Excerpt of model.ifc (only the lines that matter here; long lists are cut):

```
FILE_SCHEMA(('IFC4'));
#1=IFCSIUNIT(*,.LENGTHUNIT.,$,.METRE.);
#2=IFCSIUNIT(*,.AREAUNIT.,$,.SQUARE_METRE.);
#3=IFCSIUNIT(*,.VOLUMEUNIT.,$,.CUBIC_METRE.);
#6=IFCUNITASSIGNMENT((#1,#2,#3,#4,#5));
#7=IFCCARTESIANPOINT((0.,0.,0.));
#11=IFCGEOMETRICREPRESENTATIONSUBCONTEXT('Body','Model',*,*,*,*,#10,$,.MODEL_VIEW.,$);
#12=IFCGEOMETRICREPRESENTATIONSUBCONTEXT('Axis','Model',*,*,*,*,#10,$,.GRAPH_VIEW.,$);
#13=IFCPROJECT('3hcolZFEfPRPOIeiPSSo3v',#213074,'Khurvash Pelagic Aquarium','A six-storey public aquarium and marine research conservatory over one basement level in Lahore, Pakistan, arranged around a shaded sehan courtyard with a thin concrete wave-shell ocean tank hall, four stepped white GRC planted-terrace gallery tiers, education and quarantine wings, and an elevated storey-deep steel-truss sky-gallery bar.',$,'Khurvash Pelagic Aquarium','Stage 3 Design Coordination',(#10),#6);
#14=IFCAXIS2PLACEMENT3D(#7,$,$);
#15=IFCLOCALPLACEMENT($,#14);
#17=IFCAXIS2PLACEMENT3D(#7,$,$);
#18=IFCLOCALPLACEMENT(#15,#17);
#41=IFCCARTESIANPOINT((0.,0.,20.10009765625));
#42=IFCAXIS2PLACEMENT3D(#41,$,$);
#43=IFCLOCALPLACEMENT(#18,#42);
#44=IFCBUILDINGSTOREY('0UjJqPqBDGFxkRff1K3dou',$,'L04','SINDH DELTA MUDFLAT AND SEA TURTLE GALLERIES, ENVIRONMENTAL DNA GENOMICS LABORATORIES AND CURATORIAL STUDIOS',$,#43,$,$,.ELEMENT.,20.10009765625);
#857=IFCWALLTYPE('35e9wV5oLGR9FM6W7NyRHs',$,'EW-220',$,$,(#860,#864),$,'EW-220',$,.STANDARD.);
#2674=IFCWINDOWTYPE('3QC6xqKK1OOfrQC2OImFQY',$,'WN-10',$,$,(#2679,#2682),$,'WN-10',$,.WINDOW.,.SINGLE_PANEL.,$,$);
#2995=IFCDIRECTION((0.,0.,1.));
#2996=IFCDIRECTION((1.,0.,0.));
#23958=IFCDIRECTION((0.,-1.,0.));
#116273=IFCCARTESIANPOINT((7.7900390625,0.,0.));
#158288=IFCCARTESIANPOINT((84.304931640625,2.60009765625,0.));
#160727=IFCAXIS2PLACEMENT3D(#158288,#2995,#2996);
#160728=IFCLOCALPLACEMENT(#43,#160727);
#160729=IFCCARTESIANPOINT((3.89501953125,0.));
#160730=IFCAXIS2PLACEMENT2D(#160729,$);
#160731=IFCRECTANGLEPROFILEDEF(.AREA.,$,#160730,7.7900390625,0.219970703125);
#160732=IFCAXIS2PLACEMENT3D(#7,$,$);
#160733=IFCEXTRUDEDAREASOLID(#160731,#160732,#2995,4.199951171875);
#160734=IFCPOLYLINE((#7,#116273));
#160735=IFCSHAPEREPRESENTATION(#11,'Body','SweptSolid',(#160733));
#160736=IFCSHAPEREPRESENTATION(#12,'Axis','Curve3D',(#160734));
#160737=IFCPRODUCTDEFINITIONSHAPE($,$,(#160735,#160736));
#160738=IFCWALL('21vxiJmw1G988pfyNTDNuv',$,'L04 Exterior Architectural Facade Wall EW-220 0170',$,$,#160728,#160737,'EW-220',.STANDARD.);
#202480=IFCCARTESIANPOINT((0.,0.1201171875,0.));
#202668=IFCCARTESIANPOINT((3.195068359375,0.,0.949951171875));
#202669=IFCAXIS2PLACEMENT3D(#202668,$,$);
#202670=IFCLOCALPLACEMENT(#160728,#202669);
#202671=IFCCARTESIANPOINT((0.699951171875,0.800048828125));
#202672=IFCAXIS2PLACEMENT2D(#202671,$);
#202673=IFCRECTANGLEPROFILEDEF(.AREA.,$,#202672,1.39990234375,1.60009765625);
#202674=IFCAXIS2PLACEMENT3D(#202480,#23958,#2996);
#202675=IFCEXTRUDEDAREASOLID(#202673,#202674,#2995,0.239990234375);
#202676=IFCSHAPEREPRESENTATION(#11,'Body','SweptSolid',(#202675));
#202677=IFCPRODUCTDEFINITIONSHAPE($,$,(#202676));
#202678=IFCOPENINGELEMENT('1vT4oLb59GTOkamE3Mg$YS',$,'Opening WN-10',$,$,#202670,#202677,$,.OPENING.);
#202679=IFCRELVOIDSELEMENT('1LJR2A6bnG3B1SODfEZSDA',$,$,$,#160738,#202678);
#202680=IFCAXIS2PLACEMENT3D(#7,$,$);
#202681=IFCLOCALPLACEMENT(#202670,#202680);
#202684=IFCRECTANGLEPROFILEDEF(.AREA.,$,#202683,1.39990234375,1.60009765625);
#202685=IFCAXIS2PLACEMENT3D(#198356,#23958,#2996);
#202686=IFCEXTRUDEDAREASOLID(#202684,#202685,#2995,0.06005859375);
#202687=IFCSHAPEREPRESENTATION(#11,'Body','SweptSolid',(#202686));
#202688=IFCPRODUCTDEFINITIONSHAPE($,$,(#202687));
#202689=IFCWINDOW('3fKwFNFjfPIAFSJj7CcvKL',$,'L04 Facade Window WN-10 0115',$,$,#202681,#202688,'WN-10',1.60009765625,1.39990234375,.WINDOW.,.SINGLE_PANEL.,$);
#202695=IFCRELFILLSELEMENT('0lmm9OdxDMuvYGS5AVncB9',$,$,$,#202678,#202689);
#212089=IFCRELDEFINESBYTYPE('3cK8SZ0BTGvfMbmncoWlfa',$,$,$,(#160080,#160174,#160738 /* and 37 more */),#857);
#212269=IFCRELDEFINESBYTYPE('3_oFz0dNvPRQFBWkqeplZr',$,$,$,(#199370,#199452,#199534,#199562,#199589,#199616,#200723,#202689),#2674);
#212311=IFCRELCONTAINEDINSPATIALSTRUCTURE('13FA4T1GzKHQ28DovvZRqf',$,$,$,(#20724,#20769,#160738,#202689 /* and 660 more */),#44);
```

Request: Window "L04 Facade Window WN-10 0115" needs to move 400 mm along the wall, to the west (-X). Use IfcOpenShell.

```python
import ifcopenshell
import ifcopenshell.api.geometry
import ifcopenshell.util.placement
import ifcopenshell.util.unit

model = ifcopenshell.open("model.ifc")
unit_scale = ifcopenshell.util.unit.calculate_unit_scale(model)

window = model.by_guid("3fKwFNFjfPIAFSJj7CcvKL")
opening = window.FillsVoids[0].RelatingOpeningElement
wall = opening.VoidsElements[0].RelatingBuildingElement

wall_matrix = ifcopenshell.util.placement.get_local_placement(wall.ObjectPlacement)
shift = wall_matrix[:3, 0] * -0.4 / unit_scale
before = ifcopenshell.util.placement.get_local_placement(window.ObjectPlacement)[:3, 3].copy()

# The window is placed relative to its opening, so it follows when the opening moves.
matrix = ifcopenshell.util.placement.get_local_placement(opening.ObjectPlacement)
matrix[:3, 3] += shift
ifcopenshell.api.geometry.edit_object_placement(
    model, product=opening, matrix=matrix, is_si=False, should_transform_children=True
)

after = ifcopenshell.util.placement.get_local_placement(window.ObjectPlacement)[:3, 3]
print("window moved by", (after - before).round(3) + 0.0)

model.write("model-out.ifc")
```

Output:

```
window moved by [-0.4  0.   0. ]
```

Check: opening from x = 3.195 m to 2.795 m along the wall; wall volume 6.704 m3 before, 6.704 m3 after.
